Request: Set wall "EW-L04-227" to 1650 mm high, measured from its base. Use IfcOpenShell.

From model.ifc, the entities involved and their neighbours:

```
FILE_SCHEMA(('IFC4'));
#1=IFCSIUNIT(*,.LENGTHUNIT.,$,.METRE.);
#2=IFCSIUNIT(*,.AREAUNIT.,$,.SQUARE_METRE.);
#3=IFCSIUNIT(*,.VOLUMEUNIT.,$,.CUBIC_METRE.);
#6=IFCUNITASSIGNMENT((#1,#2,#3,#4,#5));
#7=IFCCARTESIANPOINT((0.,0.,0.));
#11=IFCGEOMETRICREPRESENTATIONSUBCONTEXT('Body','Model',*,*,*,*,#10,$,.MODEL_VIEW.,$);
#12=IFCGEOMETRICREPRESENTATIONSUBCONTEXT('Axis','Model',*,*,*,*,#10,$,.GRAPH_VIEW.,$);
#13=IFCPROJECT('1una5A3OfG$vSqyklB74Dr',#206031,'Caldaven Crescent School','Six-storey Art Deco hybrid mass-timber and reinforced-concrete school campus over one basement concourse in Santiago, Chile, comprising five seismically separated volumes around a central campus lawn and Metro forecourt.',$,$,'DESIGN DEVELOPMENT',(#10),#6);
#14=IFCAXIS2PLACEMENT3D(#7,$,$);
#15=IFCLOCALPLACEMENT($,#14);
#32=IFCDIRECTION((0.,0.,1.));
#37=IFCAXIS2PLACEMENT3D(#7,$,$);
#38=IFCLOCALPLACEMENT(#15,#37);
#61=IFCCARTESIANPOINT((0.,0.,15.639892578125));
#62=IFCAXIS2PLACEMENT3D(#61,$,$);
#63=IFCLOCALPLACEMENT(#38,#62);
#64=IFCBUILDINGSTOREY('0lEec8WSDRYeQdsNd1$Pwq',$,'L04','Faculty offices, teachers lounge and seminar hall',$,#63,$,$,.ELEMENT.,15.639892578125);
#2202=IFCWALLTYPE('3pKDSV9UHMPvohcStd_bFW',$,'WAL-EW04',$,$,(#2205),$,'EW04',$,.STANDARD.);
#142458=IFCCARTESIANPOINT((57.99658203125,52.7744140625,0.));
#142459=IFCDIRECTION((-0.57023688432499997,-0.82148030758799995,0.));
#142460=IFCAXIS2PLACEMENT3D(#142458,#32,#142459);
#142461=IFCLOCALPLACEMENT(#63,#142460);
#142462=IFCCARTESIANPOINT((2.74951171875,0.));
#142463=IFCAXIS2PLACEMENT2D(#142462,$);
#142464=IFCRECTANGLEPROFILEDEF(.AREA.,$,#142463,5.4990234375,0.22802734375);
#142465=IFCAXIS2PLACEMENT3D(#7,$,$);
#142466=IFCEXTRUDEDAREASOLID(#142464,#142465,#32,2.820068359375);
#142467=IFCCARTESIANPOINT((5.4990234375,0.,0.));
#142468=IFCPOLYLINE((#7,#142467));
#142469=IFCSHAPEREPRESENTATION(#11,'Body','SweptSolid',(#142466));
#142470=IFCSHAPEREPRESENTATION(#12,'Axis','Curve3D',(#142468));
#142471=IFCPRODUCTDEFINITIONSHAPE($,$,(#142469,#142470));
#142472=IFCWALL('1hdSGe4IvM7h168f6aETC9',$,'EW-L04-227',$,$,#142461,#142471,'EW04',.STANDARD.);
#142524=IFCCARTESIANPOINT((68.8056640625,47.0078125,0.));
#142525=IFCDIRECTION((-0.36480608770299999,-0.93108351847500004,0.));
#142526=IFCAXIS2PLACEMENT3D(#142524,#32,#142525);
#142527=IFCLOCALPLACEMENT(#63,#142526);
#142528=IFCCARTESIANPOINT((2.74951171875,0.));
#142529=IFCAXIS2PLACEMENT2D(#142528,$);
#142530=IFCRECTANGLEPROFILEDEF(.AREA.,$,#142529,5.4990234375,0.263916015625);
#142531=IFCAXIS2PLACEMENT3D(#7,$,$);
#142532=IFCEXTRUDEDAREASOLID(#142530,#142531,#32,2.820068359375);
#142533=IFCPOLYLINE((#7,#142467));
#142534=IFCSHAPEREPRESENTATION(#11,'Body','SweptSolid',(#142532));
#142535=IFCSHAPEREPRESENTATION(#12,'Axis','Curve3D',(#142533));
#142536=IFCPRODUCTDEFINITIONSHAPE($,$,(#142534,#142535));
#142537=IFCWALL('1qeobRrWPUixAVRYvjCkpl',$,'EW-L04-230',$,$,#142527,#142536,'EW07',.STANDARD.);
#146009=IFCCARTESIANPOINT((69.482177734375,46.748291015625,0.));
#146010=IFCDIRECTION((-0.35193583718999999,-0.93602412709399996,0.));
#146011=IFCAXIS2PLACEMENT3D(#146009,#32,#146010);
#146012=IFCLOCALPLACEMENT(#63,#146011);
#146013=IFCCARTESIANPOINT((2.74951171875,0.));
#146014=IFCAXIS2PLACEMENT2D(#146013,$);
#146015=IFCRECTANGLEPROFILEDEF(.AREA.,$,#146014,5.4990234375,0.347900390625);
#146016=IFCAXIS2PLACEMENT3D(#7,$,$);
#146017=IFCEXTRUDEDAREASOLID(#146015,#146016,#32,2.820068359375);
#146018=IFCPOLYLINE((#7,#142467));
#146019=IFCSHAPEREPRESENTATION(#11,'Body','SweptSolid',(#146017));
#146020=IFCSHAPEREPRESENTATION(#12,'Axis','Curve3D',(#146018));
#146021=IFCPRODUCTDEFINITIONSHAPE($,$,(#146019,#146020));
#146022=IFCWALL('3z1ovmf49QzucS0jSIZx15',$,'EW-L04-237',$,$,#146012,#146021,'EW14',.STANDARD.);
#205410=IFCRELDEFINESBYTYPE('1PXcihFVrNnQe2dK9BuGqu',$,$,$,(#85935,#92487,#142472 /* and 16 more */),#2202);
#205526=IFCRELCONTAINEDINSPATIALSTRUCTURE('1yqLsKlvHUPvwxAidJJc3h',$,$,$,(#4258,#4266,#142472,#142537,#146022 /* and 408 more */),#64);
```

```python
import ifcopenshell
import ifcopenshell.geom
import ifcopenshell.util.representation
import ifcopenshell.util.shape
import ifcopenshell.util.unit

model = ifcopenshell.open("model.ifc")
unit_scale = ifcopenshell.util.unit.calculate_unit_scale(model)
settings = ifcopenshell.geom.settings()


def volume(element):
    """Net volume in cubic metres, openings subtracted."""
    shape = ifcopenshell.geom.create_shape(settings, element)
    return ifcopenshell.util.shape.get_volume(shape.geometry)


wall = model.by_guid("1hdSGe4IvM7h168f6aETC9")
before = volume(wall)

body = ifcopenshell.util.representation.get_representation(wall, "Model", "Body")
solid = body.Items[0]
old_height = solid.Depth
solid.Depth = 1.65 / unit_scale
after = volume(wall)

print(f"height {old_height:g} -> {solid.Depth:g}, volume {before:.3f} -> {after:.3f} m3")

model.write("model_v2.ifc")
```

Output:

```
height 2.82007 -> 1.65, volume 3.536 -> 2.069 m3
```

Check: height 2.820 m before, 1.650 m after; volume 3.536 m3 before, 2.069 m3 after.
